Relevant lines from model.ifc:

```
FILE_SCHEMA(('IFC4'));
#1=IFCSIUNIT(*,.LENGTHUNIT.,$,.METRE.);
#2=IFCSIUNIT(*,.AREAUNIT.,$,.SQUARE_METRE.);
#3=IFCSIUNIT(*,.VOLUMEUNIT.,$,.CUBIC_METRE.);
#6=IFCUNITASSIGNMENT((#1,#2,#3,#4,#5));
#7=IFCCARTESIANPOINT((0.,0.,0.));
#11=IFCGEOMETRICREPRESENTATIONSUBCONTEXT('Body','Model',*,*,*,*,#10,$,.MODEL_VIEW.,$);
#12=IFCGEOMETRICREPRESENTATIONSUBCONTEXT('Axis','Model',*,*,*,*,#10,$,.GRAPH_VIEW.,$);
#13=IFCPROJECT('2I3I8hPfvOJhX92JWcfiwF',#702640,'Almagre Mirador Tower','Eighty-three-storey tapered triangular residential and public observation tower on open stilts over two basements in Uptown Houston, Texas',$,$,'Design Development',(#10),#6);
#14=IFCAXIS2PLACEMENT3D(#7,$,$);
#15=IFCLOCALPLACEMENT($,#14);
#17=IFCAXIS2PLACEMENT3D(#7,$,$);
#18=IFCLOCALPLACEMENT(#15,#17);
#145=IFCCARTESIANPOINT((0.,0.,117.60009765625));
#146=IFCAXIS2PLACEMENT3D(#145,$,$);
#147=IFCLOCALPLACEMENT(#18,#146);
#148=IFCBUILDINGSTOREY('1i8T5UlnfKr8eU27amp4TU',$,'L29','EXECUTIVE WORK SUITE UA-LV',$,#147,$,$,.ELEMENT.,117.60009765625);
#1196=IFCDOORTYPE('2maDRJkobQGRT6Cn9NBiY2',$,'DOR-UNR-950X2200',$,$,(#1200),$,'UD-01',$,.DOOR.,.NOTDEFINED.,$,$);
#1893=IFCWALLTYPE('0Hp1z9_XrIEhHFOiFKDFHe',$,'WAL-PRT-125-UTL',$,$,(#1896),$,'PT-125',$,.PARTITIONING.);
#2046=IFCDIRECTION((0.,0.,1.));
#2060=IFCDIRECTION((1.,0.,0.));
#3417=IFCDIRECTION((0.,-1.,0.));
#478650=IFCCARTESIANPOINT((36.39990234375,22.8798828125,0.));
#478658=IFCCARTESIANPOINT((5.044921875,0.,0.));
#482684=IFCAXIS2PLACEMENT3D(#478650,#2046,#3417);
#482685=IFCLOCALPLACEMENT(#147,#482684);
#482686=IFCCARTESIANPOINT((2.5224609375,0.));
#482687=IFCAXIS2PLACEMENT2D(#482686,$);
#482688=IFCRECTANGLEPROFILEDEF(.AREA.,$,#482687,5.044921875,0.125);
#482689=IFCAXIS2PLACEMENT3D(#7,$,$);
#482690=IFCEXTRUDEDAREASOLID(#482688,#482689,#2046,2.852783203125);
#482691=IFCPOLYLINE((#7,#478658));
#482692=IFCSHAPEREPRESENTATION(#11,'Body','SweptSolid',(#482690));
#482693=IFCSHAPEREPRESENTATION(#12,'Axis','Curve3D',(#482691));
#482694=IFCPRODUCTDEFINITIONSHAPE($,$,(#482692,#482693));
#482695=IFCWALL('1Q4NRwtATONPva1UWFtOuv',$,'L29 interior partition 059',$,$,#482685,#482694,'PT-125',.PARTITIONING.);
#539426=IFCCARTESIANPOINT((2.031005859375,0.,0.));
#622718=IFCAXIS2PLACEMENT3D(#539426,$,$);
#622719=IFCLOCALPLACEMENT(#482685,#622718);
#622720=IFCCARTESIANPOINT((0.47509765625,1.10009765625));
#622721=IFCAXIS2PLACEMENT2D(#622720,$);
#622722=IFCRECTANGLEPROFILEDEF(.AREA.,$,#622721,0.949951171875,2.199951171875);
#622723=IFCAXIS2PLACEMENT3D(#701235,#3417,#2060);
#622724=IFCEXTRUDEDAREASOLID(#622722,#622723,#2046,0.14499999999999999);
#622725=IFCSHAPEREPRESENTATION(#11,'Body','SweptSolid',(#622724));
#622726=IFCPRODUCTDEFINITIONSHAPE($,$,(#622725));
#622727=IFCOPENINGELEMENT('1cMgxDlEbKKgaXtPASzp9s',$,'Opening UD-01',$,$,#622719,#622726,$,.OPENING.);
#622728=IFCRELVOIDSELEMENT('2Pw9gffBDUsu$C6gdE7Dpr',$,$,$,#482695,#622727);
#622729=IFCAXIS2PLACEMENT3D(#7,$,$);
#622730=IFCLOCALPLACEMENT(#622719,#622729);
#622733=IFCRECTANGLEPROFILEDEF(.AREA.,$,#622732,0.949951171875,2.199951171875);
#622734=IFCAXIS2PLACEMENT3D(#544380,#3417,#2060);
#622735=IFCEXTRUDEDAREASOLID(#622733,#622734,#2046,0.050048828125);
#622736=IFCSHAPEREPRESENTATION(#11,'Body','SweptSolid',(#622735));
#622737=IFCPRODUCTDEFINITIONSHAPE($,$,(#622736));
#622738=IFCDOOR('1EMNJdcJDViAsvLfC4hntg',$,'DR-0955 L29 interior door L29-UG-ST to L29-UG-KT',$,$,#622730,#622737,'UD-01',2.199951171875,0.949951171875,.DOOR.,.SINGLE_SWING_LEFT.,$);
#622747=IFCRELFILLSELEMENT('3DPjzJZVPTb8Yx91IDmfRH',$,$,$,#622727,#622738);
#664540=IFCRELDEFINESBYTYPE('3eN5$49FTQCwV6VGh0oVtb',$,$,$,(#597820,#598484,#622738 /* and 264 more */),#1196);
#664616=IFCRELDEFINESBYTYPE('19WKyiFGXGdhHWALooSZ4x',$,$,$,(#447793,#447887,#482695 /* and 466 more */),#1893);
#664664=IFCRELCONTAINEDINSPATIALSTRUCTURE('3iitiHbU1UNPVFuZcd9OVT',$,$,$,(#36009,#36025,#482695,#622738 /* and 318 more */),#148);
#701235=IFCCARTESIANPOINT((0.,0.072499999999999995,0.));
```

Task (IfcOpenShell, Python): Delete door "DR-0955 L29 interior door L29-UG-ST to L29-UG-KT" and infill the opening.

```python
import ifcopenshell
import ifcopenshell.api.feature
import ifcopenshell.api.root
import ifcopenshell.geom
import ifcopenshell.util.shape

model = ifcopenshell.open("model.ifc")
settings = ifcopenshell.geom.settings()


def volume(element):
    """Net volume in cubic metres, openings subtracted."""
    shape = ifcopenshell.geom.create_shape(settings, element)
    return ifcopenshell.util.shape.get_volume(shape.geometry)


door = model.by_guid("1EMNJdcJDViAsvLfC4hntg")
opening = door.FillsVoids[0].RelatingOpeningElement
wall = opening.VoidsElements[0].RelatingBuildingElement
before = volume(wall)

ifcopenshell.api.root.remove_product(model, product=door)
ifcopenshell.api.feature.remove_feature(model, feature=opening)

after = volume(wall)

print(f"wall volume {before:.3f} -> {after:.3f} m3")

model.write("model-out.ifc")
```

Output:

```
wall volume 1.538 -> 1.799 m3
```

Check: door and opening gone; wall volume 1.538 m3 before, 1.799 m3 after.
